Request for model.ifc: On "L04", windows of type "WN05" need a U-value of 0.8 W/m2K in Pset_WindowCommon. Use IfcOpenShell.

First a look at what the model holds.

```python
import ifcopenshell
import ifcopenshell.util.element

model = ifcopenshell.open("model.ifc")
print(model.schema)
storey = next(s for s in model.by_type("IfcBuildingStorey") if s.Name == "L04")
windows = [e for e in ifcopenshell.util.element.get_decomposition(storey) if e.is_a("IfcWindow")]
seen = {}
for e in windows:
    element_type = ifcopenshell.util.element.get_type(e)
    key = (element_type.Name if element_type != e and element_type else None, ifcopenshell.util.element.get_pset(e, "Pset_WindowCommon", "ThermalTransmittance"))
    seen[key] = seen.get(key, 0) + 1
for (name, value), count in sorted(seen.items(), key=str):
    print(count, "x", name, "|", value)
```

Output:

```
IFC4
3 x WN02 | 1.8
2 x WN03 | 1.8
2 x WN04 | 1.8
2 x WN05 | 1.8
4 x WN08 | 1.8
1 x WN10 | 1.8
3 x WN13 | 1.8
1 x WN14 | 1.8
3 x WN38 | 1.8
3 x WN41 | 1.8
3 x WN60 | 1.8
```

```python
import ifcopenshell
import ifcopenshell.api.pset
import ifcopenshell.util.element

model = ifcopenshell.open("model.ifc")

storey = next(s for s in model.by_type("IfcBuildingStorey") if s.Name == "L04")
windows = [e for e in ifcopenshell.util.element.get_decomposition(storey) if e.is_a("IfcWindow")]

count = 0
for e in windows:
    element_type = ifcopenshell.util.element.get_type(e)
    if element_type in (None, e) or element_type.Name != "WN05":
        continue
    # add_pset returns the element's existing set when there is one.
    pset = ifcopenshell.api.pset.add_pset(model, product=e, name="Pset_WindowCommon")
    ifcopenshell.api.pset.edit_pset(model, pset=pset, properties={"ThermalTransmittance": 0.8})
    count += 1

print(count, "windows updated")

model.write("model_updated.ifc")
```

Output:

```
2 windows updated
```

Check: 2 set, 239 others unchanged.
